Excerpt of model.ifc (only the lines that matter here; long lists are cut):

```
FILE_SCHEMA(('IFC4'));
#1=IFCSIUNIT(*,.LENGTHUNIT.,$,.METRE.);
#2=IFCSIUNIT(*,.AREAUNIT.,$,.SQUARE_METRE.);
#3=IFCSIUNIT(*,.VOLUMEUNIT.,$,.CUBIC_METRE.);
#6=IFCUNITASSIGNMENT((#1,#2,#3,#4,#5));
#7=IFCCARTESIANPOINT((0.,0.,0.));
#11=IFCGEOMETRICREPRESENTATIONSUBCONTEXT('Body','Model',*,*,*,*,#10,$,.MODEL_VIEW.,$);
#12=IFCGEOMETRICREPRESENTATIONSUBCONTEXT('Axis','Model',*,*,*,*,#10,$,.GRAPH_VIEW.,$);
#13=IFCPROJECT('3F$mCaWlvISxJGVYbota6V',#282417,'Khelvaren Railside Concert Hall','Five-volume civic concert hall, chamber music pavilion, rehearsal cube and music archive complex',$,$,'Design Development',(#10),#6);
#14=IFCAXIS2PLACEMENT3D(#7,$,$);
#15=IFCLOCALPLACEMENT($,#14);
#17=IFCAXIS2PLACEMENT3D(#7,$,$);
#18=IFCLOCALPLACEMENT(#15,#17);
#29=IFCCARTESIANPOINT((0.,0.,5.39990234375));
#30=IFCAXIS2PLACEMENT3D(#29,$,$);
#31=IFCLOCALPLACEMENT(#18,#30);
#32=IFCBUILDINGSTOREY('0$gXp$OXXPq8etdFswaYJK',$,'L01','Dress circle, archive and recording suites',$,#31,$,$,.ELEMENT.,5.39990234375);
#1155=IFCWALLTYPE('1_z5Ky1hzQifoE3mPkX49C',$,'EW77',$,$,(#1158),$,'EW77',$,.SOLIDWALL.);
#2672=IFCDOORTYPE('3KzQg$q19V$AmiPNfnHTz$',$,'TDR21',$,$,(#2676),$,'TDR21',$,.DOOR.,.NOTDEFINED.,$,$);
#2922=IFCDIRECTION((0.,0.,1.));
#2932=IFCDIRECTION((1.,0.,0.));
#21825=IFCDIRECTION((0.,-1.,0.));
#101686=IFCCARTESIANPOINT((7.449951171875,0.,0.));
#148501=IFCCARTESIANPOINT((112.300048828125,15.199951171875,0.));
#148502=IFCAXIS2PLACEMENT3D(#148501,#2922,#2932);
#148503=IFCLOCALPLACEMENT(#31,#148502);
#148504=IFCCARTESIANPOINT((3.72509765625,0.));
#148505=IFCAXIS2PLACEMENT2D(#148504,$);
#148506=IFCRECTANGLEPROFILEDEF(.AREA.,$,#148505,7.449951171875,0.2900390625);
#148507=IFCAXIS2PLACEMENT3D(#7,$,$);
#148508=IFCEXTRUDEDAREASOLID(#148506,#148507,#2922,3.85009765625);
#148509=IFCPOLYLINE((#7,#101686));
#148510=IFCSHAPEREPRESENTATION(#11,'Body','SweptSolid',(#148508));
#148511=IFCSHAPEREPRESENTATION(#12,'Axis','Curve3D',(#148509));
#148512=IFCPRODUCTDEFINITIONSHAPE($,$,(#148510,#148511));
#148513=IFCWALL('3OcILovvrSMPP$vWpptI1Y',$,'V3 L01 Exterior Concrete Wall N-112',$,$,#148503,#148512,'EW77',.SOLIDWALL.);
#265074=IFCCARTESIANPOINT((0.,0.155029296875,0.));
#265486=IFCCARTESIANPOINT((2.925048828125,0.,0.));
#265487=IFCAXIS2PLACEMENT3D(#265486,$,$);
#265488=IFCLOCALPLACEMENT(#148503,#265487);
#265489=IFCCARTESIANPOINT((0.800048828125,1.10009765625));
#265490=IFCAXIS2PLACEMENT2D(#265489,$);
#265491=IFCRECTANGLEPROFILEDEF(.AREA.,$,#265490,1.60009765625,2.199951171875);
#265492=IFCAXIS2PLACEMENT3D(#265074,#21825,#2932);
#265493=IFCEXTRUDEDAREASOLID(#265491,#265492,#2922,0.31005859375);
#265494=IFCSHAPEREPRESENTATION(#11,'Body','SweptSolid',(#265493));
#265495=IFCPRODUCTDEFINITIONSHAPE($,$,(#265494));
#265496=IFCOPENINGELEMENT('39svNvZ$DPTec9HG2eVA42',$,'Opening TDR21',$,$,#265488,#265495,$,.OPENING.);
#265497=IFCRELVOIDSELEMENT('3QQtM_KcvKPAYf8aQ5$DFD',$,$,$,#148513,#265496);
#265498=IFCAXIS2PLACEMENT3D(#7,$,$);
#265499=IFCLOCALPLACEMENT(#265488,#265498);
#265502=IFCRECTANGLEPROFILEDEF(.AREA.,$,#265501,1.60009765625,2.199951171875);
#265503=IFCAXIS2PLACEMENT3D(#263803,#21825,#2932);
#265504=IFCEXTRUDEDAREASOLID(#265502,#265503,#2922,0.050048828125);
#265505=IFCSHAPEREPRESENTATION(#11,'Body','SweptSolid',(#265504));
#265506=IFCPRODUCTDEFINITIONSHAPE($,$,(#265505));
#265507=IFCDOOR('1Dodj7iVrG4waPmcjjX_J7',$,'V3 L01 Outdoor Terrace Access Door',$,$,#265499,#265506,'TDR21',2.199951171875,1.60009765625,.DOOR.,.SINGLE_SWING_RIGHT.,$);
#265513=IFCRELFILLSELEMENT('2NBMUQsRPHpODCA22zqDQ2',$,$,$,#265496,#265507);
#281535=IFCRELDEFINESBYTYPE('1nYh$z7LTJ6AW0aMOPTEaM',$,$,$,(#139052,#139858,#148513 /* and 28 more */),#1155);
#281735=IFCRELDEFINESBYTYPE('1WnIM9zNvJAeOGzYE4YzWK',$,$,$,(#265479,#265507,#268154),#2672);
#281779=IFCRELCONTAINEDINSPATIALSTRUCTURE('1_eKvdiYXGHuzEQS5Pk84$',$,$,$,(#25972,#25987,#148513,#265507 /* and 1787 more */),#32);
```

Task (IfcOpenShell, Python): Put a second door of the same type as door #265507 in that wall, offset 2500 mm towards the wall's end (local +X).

```python
import ifcopenshell
import ifcopenshell.api.feature
import ifcopenshell.api.geometry
import ifcopenshell.api.root
import ifcopenshell.geom
import ifcopenshell.util.element
import ifcopenshell.util.placement
import ifcopenshell.util.shape
import ifcopenshell.util.unit

model = ifcopenshell.open("model.ifc")
unit_scale = ifcopenshell.util.unit.calculate_unit_scale(model)
settings = ifcopenshell.geom.settings()


def volume(element):
    """Net volume in cubic metres, openings subtracted."""
    shape = ifcopenshell.geom.create_shape(settings, element)
    return ifcopenshell.util.shape.get_volume(shape.geometry)


door = model.by_guid("1Dodj7iVrG4waPmcjjX_J7")
opening = door.FillsVoids[0].RelatingOpeningElement
wall = opening.VoidsElements[0].RelatingBuildingElement
before = volume(wall)
shift = ifcopenshell.util.placement.get_local_placement(wall.ObjectPlacement)[:3, 0] * 2.5 / unit_scale

# copy_class copies the void relationship, type, container and properties, but no geometry.
new_opening = ifcopenshell.api.root.copy_class(model, product=opening)
new_opening.Representation = ifcopenshell.util.element.copy_deep(
    model, opening.Representation, exclude=["IfcGeometricRepresentationContext", "IfcRepresentationMap"]
)
new_door = ifcopenshell.api.root.copy_class(model, product=door)
new_door.Representation = ifcopenshell.util.element.copy_deep(
    model, door.Representation, exclude=["IfcGeometricRepresentationContext", "IfcRepresentationMap"]
)
new_door.Tag = None
ifcopenshell.api.feature.add_filling(model, opening=new_opening, element=new_door)

for old, new in ((opening, new_opening), (door, new_door)):
    matrix = ifcopenshell.util.placement.get_local_placement(old.ObjectPlacement)
    matrix[:3, 3] += shift
    ifcopenshell.api.geometry.edit_object_placement(model, product=new, matrix=matrix, is_si=False)

after = volume(wall)

print(f"wall volume {before:.3f} -> {after:.3f} m3")

model.write("model_updated.ifc")
```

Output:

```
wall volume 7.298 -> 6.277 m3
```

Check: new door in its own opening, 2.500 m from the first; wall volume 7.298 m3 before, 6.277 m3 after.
